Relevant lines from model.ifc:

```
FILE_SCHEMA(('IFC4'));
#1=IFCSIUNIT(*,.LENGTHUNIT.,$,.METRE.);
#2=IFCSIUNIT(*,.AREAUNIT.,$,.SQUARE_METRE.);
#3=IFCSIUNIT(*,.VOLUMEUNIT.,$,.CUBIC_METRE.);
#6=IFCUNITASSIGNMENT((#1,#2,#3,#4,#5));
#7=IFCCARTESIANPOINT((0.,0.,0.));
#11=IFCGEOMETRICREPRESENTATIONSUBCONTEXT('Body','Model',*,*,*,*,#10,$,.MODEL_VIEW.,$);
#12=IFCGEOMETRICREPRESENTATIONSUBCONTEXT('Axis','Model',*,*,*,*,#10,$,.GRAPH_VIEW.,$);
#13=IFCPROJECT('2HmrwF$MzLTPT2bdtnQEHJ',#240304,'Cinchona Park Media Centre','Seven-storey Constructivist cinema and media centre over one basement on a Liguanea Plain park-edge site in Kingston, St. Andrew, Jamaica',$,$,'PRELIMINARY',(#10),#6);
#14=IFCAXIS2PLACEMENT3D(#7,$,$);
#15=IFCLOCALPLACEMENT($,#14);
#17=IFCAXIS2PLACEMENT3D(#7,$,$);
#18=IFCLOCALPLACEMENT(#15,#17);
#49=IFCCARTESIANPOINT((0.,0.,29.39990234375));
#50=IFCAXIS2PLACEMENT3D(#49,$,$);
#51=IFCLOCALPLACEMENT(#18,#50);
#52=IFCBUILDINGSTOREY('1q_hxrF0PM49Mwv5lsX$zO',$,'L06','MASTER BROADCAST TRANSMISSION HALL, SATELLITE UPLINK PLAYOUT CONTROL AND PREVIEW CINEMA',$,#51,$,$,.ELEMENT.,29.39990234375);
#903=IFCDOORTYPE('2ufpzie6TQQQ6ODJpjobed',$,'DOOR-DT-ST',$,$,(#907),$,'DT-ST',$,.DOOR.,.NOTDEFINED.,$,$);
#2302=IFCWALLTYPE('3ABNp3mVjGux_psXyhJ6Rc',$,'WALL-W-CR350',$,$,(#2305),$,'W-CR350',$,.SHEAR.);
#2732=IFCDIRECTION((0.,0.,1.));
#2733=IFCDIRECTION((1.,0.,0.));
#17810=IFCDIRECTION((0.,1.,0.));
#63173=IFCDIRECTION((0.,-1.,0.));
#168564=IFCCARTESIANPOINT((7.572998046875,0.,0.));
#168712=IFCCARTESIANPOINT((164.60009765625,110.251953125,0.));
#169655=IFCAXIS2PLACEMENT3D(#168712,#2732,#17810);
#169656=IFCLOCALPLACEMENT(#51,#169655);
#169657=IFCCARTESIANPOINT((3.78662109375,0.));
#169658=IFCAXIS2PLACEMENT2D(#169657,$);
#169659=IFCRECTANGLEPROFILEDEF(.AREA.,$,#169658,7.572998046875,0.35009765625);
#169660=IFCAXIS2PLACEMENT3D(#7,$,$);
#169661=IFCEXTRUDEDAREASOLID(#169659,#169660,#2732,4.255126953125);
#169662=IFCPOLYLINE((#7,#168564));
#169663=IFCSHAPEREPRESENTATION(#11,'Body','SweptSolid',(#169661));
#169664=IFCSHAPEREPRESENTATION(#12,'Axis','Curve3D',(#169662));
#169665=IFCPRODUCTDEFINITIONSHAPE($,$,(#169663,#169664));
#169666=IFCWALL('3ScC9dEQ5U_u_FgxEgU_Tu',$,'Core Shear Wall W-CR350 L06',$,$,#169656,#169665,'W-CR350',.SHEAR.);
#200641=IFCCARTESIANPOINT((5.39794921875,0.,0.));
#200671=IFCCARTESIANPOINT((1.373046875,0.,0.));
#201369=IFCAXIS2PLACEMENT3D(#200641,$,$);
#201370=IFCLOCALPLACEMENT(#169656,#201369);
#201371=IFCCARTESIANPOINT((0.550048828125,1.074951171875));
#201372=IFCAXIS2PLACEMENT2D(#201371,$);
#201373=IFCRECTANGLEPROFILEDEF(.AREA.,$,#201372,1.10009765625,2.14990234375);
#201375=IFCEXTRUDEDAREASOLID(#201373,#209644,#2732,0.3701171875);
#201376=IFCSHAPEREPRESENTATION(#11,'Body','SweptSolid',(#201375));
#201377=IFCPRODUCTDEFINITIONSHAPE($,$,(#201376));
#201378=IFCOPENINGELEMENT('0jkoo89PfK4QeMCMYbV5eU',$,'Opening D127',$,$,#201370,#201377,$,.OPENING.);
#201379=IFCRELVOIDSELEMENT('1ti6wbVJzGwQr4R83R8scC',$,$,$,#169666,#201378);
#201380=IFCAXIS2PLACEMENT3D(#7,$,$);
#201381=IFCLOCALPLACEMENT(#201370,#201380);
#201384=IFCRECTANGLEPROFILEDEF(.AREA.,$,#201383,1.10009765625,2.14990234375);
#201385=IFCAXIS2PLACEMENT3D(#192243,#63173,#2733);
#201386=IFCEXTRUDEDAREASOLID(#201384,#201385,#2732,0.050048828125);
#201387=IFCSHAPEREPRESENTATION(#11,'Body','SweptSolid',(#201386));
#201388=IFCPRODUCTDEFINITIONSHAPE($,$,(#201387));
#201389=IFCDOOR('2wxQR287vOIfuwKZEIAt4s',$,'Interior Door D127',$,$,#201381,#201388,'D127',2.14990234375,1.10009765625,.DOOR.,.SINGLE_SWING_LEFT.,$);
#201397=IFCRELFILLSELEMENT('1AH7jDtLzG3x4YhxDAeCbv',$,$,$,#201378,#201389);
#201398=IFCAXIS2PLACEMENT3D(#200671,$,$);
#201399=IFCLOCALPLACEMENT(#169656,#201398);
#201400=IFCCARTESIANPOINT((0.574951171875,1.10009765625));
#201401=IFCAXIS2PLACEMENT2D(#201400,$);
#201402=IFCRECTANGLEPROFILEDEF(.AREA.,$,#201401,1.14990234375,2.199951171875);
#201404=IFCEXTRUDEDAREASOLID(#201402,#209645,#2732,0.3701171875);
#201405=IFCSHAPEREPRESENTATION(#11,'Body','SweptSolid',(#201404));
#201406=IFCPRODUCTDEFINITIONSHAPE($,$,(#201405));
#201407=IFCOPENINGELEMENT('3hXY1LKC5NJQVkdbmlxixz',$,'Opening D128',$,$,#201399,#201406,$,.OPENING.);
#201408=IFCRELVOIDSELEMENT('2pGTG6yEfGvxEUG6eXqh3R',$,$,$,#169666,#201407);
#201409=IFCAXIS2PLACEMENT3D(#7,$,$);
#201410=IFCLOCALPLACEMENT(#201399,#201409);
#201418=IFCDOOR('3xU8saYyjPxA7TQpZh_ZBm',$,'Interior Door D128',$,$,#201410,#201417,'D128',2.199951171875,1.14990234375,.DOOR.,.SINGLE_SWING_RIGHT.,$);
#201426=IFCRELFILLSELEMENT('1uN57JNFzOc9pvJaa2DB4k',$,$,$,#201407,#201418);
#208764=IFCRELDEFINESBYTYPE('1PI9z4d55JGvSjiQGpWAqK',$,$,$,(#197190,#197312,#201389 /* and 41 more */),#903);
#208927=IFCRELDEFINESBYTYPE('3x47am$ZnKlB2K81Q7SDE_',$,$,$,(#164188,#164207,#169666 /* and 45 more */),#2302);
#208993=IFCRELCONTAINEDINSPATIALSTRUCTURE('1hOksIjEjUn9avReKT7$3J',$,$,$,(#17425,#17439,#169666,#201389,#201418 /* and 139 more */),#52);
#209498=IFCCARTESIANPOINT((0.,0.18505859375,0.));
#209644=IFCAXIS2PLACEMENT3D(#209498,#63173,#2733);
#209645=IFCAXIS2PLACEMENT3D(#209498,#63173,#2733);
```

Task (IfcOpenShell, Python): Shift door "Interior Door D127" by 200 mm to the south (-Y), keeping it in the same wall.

```python
import ifcopenshell
import ifcopenshell.api.geometry
import ifcopenshell.util.placement
import ifcopenshell.util.unit

model = ifcopenshell.open("model.ifc")
unit_scale = ifcopenshell.util.unit.calculate_unit_scale(model)

door = model.by_guid("2wxQR287vOIfuwKZEIAt4s")
opening = door.FillsVoids[0].RelatingOpeningElement
wall = opening.VoidsElements[0].RelatingBuildingElement

wall_matrix = ifcopenshell.util.placement.get_local_placement(wall.ObjectPlacement)
shift = wall_matrix[:3, 0] * -0.2 / unit_scale
before = ifcopenshell.util.placement.get_local_placement(door.ObjectPlacement)[:3, 3].copy()

# The door is placed relative to its opening, so it follows when the opening moves.
matrix = ifcopenshell.util.placement.get_local_placement(opening.ObjectPlacement)
matrix[:3, 3] += shift
ifcopenshell.api.geometry.edit_object_placement(
    model, product=opening, matrix=matrix, is_si=False, should_transform_children=True
)

after = ifcopenshell.util.placement.get_local_placement(door.ObjectPlacement)[:3, 3]
print("door moved by", (after - before).round(3) + 0.0)

model.write("model_v2.ifc")
```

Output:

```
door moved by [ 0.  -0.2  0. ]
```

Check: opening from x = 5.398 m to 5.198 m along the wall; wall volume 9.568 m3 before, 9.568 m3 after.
